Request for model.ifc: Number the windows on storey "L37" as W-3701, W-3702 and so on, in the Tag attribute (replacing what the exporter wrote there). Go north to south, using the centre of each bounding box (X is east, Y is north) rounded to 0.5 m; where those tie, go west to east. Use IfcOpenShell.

First a look at what the model holds.

```python
import ifcopenshell
import ifcopenshell.util.element
import ifcopenshell.util.placement

model = ifcopenshell.open("model.ifc")
print(model.schema)
storey = next(s for s in model.by_type("IfcBuildingStorey") if s.Name == "L37")
windows = [e for e in ifcopenshell.util.element.get_decomposition(storey) if e.is_a("IfcWindow")]
for e in sorted(windows, key=lambda e: e.id()):
    origin = ifcopenshell.util.placement.get_local_placement(e.ObjectPlacement)[:3, 3]
    print(e.id(), e.Tag, e.Name, origin.round(2) + 0.0, sep=" | ")
```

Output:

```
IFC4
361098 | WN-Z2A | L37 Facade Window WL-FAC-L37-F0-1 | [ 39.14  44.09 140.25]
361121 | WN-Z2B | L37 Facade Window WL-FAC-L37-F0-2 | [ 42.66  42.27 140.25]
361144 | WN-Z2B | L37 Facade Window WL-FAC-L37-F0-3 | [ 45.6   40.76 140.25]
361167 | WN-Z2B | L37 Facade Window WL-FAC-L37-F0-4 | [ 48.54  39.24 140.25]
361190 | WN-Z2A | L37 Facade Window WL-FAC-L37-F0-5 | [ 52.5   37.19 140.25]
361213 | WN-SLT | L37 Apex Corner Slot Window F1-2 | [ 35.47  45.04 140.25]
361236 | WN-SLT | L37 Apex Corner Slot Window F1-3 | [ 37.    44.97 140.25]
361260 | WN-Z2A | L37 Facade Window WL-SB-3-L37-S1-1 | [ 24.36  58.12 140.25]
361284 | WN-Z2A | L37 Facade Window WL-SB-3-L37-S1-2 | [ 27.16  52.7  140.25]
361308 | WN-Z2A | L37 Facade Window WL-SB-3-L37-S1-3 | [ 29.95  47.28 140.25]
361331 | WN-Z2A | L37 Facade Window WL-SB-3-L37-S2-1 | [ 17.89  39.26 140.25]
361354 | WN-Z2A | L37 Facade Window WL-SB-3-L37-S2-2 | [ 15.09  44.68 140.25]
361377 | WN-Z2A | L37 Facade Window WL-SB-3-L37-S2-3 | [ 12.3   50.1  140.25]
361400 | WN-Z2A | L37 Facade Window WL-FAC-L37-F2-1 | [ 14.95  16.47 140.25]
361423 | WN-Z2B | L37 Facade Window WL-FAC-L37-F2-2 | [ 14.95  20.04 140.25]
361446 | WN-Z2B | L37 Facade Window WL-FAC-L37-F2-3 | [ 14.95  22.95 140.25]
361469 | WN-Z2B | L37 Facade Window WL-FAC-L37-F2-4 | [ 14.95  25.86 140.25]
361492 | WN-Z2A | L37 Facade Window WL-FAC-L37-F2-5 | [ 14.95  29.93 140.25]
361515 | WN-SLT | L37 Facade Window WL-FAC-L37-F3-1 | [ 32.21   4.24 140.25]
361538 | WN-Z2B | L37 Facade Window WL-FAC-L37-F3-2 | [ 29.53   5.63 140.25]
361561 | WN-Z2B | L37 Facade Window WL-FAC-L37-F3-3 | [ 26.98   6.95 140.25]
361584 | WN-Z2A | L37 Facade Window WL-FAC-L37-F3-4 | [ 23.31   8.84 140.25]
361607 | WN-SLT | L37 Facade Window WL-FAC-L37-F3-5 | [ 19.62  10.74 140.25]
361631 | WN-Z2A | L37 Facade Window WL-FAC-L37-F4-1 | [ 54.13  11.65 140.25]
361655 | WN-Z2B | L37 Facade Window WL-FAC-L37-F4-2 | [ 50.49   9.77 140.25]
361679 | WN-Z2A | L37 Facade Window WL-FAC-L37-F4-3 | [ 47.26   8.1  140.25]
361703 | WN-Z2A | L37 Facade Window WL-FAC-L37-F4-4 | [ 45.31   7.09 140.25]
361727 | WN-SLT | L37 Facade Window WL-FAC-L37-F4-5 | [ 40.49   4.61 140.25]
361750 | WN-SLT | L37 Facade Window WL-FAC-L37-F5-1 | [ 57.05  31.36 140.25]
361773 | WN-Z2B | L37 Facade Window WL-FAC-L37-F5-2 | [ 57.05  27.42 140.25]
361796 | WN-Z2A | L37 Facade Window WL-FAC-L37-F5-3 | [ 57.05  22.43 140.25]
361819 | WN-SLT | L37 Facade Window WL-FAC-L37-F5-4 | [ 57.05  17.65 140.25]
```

```python
import ifcopenshell
import ifcopenshell.geom
import ifcopenshell.util.element
import ifcopenshell.util.shape

model = ifcopenshell.open("model.ifc")
settings = ifcopenshell.geom.settings()
settings.set("use-world-coords", True)


def centre(element):
    shape = ifcopenshell.geom.create_shape(settings, element)
    return ifcopenshell.util.shape.get_bbox_centroid(shape.geometry)


storey = next(s for s in model.by_type("IfcBuildingStorey") if s.Name == "L37")
windows = [e for e in ifcopenshell.util.element.get_decomposition(storey) if e.is_a("IfcWindow")]

# Insertion points can sit at a corner or the storey origin, so sort by the geometry (in metres).
centres = {e: centre(e) for e in windows}
windows.sort(key=lambda e: (-round(centres[e][1] / 0.5), centres[e][0]))

for i, e in enumerate(windows, start=1):
    number = f"W-37{i:02d}"
    e.Tag = number
    print(e.id(), number)

model.write("model-out.ifc")
```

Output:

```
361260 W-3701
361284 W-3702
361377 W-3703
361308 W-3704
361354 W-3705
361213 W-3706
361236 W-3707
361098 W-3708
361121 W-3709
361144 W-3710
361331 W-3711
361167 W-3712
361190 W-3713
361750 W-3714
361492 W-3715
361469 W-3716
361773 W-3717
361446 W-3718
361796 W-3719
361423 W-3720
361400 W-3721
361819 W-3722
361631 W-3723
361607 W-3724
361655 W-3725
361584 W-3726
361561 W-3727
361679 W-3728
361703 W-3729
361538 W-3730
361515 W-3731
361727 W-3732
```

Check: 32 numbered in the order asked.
